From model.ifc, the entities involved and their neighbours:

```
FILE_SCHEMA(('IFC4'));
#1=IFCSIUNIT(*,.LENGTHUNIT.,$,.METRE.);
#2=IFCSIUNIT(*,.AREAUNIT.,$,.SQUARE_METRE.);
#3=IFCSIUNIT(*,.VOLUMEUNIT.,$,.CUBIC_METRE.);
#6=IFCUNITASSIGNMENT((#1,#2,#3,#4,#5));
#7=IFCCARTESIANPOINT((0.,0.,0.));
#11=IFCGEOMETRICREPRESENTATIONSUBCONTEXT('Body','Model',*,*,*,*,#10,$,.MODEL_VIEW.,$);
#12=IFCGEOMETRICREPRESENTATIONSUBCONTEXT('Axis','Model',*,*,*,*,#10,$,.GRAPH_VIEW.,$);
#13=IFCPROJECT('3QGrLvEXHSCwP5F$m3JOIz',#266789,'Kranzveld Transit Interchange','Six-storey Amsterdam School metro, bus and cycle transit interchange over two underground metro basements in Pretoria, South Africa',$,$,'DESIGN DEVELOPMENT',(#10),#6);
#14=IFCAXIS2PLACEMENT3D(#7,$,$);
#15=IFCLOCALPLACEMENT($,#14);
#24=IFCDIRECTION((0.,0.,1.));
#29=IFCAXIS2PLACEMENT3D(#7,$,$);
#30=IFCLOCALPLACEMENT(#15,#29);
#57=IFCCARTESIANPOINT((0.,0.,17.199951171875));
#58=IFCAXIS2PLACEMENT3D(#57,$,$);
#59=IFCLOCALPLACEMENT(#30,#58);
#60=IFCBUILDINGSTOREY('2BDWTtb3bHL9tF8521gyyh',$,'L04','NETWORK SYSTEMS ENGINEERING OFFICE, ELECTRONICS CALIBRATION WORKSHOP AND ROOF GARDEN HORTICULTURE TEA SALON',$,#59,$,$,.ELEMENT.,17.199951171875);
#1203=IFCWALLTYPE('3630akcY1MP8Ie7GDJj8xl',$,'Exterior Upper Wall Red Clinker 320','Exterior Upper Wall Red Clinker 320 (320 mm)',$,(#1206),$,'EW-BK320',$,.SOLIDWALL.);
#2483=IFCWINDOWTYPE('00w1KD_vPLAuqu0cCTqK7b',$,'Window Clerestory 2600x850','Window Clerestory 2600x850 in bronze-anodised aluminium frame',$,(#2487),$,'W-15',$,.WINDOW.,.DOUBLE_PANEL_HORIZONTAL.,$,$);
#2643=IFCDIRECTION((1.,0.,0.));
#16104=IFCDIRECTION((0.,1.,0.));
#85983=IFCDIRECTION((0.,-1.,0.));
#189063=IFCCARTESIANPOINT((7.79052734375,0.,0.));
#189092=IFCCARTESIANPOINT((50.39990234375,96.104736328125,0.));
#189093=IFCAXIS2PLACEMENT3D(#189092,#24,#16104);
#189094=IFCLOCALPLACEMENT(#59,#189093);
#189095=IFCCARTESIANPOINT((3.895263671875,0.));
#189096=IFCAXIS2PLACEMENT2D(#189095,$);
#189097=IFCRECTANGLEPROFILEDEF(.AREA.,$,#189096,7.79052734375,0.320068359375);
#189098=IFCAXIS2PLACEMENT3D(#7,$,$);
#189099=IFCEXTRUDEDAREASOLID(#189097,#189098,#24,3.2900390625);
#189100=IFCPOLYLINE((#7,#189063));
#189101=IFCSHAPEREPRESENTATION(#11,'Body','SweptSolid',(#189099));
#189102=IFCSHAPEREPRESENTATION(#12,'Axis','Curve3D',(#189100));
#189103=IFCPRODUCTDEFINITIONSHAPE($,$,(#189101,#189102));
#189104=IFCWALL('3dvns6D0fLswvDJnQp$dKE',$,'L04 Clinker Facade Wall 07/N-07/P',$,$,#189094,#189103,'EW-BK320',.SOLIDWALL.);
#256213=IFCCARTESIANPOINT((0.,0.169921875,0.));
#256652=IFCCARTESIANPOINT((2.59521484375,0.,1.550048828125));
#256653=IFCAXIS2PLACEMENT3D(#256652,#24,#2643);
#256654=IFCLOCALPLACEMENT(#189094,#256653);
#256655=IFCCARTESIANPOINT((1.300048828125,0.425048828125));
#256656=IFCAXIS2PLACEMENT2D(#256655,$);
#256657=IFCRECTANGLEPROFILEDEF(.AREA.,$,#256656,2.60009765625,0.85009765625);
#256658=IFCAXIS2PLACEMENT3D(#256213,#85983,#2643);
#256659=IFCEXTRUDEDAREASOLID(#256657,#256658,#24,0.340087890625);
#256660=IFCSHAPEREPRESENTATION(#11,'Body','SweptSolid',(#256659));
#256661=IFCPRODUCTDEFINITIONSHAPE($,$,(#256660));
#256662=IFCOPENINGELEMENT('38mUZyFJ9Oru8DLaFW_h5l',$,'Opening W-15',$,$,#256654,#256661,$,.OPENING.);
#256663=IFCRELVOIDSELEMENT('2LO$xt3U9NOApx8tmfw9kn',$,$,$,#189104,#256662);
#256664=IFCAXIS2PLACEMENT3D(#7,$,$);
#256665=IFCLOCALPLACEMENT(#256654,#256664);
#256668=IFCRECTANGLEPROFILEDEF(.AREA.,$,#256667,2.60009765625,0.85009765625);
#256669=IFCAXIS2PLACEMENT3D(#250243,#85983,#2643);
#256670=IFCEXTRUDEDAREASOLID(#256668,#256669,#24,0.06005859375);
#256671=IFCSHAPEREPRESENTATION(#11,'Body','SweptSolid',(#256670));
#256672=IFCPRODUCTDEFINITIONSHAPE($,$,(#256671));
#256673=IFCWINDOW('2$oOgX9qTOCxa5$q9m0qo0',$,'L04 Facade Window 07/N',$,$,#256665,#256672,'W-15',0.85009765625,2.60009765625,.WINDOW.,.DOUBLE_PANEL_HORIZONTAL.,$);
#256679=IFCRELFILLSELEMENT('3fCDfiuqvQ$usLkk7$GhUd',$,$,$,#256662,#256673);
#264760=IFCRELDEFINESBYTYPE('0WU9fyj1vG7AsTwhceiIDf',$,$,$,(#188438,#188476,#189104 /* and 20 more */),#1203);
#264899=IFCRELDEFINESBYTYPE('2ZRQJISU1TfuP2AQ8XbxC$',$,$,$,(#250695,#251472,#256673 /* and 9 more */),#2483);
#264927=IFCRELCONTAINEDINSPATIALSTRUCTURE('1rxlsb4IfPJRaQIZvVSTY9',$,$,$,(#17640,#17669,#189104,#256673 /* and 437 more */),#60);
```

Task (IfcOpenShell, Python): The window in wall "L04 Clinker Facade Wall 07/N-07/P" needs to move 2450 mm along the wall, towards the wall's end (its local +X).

```python
import ifcopenshell
import ifcopenshell.api.geometry
import ifcopenshell.util.placement

model = ifcopenshell.open("model.ifc")

window = model.by_guid("2$oOgX9qTOCxa5$q9m0qo0")
opening = window.FillsVoids[0].RelatingOpeningElement
wall = opening.VoidsElements[0].RelatingBuildingElement

wall_matrix = ifcopenshell.util.placement.get_local_placement(wall.ObjectPlacement)
shift = wall_matrix[:3, 0] * 2.45
before = ifcopenshell.util.placement.get_local_placement(window.ObjectPlacement)[:3, 3].copy()

# The window is placed relative to its opening, so it follows when the opening moves.
matrix = ifcopenshell.util.placement.get_local_placement(opening.ObjectPlacement)
matrix[:3, 3] += shift
ifcopenshell.api.geometry.edit_object_placement(
    model, product=opening, matrix=matrix, is_si=False, should_transform_children=True
)

after = ifcopenshell.util.placement.get_local_placement(window.ObjectPlacement)[:3, 3]
print("window moved by", (after - before).round(3) + 0.0)

model.write("model_v2.ifc")
```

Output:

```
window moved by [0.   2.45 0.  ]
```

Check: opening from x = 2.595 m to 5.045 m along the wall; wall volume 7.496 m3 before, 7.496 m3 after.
